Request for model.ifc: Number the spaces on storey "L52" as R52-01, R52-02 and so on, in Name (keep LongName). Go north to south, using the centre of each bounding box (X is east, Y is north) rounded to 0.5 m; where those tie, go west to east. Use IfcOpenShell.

First a look at what the model holds.

```python
import ifcopenshell
import ifcopenshell.util.element
import ifcopenshell.util.placement

model = ifcopenshell.open("model.ifc")
print(model.schema)
storey = next(s for s in model.by_type("IfcBuildingStorey") if s.Name == "L52")
spaces = [e for e in ifcopenshell.util.element.get_decomposition(storey) if e.is_a("IfcSpace")]
for e in sorted(spaces, key=lambda e: e.id()):
    origin = ifcopenshell.util.placement.get_local_placement(e.ObjectPlacement)[:3, 3]
    print(e.id(), e.Name, e.LongName, origin.round(2) + 0.0, sep=" | ")
```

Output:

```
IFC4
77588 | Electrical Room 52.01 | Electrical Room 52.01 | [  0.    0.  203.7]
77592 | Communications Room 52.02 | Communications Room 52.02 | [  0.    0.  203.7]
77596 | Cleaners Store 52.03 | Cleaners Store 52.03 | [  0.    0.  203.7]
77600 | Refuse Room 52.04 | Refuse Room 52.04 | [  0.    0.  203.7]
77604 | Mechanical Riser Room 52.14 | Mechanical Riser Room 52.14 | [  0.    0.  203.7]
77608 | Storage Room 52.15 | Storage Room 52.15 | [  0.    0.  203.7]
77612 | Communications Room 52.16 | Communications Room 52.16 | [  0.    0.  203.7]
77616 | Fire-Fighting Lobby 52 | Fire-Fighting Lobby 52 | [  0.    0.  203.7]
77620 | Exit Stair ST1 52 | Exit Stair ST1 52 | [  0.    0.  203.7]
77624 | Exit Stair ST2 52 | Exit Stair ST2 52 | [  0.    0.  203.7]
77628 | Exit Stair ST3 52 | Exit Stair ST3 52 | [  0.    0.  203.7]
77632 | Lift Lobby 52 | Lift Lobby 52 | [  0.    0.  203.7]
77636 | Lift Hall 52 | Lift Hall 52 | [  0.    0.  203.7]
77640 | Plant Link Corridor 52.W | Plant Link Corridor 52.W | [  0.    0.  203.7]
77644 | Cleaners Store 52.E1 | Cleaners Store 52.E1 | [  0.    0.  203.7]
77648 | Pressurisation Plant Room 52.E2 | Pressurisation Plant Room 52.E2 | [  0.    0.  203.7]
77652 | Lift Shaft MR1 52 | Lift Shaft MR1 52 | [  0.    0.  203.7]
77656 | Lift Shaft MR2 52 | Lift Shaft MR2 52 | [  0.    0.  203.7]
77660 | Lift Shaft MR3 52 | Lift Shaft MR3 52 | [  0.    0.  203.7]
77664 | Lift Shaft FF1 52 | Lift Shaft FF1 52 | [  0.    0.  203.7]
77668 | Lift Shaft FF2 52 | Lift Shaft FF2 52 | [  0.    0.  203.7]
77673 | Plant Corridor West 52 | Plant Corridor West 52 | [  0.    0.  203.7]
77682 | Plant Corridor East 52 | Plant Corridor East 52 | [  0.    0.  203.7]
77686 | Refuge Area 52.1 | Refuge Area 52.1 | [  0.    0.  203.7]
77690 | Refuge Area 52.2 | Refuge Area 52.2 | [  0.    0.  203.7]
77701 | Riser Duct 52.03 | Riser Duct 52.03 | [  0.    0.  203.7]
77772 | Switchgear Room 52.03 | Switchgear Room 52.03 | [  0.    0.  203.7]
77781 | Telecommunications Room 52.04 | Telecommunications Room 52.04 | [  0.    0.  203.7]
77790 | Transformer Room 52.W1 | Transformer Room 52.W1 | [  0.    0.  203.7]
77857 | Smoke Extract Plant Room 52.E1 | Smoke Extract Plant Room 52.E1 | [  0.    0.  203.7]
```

```python
import ifcopenshell
import ifcopenshell.geom
import ifcopenshell.util.element
import ifcopenshell.util.shape

model = ifcopenshell.open("model.ifc")
settings = ifcopenshell.geom.settings()
settings.set("use-world-coords", True)


def centre(element):
    shape = ifcopenshell.geom.create_shape(settings, element)
    return ifcopenshell.util.shape.get_bbox_centroid(shape.geometry)


storey = next(s for s in model.by_type("IfcBuildingStorey") if s.Name == "L52")
spaces = [e for e in ifcopenshell.util.element.get_decomposition(storey) if e.is_a("IfcSpace")]

# Insertion points can sit at a corner or the storey origin, so sort by the geometry (in metres).
centres = {e: centre(e) for e in spaces}
spaces.sort(key=lambda e: (-round(centres[e][1] / 0.5), centres[e][0]))

for i, e in enumerate(spaces, start=1):
    number = f"R52-{i:02d}"
    e.Name = number
    print(e.id(), number)

model.write("model_updated.ifc")
```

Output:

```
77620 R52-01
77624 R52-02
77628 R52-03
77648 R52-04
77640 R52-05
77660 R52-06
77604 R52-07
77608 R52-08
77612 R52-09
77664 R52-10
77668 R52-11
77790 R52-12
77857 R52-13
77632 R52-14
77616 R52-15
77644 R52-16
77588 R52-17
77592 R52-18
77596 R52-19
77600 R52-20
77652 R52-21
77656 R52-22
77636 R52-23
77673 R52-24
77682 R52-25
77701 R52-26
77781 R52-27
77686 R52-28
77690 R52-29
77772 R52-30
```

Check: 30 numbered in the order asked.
